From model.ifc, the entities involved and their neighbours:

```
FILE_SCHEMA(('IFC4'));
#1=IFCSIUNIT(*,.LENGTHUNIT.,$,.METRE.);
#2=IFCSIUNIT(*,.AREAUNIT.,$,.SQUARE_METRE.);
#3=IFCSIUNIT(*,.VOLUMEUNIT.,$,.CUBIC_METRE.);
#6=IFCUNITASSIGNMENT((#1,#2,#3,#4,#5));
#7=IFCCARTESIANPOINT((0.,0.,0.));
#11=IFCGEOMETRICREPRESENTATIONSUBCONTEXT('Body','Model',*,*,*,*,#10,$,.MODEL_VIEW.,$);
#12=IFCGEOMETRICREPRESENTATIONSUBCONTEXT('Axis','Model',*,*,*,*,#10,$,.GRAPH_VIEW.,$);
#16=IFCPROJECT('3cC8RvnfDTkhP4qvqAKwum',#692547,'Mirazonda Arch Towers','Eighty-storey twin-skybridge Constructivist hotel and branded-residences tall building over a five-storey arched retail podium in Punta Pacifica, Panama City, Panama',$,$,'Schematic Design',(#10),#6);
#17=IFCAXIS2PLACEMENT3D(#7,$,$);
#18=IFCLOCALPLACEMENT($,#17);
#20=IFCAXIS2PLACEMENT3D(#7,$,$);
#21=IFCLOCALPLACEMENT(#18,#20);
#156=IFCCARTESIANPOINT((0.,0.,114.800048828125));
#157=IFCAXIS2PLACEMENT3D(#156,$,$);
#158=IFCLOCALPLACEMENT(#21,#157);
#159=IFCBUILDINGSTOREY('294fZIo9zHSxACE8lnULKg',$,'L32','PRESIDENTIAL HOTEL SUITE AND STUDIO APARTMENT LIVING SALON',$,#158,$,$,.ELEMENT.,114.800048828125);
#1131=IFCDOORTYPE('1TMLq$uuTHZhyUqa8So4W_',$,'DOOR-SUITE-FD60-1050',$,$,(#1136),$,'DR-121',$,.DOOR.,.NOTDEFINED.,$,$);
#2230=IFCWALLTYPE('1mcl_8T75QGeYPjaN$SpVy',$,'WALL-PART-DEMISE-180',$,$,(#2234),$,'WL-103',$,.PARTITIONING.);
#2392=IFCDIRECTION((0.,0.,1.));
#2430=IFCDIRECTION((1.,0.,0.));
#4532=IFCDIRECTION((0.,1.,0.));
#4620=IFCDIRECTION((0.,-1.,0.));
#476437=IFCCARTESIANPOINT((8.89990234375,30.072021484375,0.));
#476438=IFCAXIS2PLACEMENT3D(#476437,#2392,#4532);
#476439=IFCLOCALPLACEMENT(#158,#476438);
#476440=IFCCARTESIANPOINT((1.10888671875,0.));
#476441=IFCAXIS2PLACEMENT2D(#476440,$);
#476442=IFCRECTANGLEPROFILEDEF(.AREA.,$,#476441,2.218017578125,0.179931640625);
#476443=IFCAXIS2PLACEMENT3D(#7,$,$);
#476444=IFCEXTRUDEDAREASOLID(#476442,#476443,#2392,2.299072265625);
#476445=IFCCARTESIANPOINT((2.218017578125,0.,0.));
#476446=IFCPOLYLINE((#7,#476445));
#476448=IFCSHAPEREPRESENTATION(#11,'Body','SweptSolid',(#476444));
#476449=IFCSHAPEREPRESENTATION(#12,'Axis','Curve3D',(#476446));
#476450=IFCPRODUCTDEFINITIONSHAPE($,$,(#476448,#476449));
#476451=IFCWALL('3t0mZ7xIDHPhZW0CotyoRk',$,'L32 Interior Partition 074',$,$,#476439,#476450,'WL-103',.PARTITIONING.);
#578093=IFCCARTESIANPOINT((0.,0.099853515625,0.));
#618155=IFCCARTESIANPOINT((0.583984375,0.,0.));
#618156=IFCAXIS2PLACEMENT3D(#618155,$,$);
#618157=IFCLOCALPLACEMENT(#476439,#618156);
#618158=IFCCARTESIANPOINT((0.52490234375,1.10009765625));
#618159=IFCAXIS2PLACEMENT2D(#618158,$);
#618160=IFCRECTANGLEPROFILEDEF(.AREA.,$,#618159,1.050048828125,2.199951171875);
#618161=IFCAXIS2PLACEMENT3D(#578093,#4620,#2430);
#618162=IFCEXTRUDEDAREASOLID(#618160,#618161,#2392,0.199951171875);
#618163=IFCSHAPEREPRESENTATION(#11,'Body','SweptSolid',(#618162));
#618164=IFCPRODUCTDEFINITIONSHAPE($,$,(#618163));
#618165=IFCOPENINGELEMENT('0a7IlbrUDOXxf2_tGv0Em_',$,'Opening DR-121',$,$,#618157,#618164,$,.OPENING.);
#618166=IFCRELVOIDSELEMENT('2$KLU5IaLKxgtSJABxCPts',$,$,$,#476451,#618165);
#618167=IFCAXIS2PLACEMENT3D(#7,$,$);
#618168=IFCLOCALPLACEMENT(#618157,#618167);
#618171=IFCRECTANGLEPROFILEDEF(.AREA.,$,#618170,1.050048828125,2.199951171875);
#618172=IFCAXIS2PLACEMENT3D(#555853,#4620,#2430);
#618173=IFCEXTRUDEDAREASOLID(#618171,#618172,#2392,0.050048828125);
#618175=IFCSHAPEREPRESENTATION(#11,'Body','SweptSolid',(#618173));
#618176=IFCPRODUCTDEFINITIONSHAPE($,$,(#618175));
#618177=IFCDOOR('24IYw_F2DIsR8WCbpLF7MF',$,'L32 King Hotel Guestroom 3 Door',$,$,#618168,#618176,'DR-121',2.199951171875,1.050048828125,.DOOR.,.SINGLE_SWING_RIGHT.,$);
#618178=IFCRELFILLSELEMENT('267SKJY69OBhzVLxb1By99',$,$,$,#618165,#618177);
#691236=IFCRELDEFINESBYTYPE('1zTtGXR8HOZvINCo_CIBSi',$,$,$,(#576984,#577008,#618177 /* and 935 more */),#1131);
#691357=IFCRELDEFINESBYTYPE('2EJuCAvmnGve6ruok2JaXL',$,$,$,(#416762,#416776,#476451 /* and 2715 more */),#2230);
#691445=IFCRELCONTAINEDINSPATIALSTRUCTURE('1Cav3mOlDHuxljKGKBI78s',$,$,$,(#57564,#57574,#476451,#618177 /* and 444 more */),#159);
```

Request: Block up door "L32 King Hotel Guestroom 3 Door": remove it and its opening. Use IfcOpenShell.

```python
import ifcopenshell
import ifcopenshell.api.feature
import ifcopenshell.api.root
import ifcopenshell.geom
import ifcopenshell.util.shape

model = ifcopenshell.open("model.ifc")
settings = ifcopenshell.geom.settings()


def volume(element):
    """Net volume in cubic metres, openings subtracted."""
    shape = ifcopenshell.geom.create_shape(settings, element)
    return ifcopenshell.util.shape.get_volume(shape.geometry)


door = model.by_guid("24IYw_F2DIsR8WCbpLF7MF")
opening = door.FillsVoids[0].RelatingOpeningElement
wall = opening.VoidsElements[0].RelatingBuildingElement
before = volume(wall)

ifcopenshell.api.root.remove_product(model, product=door)
ifcopenshell.api.feature.remove_feature(model, feature=opening)

after = volume(wall)

print(f"wall volume {before:.3f} -> {after:.3f} m3")

model.write("model_updated.ifc")
```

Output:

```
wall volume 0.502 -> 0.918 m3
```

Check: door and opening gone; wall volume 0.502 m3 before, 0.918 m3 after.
